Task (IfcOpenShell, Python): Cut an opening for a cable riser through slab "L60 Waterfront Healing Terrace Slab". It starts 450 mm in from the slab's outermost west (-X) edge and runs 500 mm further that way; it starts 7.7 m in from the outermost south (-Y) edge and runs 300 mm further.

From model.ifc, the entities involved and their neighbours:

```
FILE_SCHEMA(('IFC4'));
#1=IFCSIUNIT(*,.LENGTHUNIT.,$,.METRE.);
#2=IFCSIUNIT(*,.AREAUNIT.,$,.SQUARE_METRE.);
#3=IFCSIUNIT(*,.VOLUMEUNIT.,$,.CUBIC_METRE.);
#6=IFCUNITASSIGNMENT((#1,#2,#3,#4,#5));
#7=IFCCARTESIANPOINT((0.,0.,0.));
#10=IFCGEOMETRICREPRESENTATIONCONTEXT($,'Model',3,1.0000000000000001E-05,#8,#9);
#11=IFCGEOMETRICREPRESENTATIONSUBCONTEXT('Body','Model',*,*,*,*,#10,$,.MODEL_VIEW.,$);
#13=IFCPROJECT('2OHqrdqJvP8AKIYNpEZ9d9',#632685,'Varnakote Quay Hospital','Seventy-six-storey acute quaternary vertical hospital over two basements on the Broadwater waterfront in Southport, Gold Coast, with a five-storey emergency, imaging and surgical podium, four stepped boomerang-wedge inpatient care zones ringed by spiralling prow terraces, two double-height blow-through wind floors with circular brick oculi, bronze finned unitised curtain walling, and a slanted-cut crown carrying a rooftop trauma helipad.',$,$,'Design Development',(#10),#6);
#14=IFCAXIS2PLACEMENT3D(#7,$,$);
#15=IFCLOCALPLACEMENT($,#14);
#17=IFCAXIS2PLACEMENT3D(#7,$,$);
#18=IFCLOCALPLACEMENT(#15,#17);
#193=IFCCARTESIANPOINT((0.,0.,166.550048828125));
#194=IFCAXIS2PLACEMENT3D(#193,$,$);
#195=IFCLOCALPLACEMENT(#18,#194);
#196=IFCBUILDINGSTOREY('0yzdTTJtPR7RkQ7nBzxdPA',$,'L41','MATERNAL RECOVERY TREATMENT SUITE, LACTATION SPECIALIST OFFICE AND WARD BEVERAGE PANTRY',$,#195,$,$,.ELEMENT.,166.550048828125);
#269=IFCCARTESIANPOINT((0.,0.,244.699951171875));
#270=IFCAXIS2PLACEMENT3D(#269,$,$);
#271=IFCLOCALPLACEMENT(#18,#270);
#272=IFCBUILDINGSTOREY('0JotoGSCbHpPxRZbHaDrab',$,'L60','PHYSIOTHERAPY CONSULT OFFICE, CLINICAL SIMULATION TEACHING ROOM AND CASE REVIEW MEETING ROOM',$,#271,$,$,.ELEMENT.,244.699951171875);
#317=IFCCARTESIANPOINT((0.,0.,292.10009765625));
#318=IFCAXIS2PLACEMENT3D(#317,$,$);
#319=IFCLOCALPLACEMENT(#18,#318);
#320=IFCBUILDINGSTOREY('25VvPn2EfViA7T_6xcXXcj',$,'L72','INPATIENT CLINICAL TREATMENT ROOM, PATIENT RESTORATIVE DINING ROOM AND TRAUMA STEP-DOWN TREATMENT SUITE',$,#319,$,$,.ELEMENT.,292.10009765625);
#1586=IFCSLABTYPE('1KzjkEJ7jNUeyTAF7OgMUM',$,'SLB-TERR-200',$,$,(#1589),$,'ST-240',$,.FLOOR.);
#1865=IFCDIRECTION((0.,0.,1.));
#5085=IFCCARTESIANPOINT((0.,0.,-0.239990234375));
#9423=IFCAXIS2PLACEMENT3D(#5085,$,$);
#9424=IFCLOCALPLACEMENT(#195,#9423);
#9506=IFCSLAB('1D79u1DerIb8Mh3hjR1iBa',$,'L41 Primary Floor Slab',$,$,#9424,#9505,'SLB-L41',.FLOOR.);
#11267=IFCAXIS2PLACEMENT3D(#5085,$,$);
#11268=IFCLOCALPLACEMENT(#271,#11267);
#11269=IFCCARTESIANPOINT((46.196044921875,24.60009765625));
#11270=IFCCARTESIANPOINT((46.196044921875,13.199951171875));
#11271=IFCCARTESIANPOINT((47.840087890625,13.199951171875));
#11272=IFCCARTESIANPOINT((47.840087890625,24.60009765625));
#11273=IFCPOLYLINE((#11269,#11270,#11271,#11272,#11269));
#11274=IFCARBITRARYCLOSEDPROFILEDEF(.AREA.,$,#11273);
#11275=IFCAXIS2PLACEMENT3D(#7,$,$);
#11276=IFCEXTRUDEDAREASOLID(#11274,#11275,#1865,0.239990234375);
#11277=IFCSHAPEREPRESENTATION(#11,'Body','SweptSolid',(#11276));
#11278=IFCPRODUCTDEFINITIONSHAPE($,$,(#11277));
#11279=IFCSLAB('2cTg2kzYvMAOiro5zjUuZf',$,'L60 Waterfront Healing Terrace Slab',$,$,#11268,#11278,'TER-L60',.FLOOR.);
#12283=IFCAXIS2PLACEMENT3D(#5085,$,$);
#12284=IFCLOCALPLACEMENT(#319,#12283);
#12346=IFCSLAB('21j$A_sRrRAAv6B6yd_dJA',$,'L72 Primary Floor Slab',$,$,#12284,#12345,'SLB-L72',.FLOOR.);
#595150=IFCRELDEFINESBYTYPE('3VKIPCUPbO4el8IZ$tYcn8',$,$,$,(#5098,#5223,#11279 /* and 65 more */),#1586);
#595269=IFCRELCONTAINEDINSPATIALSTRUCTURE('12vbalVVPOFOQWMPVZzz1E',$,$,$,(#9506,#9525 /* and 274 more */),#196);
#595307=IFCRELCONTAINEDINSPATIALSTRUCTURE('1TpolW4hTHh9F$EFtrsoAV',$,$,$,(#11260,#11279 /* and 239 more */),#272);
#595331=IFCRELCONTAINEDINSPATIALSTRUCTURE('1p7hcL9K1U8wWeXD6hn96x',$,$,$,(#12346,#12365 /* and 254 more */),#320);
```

```python
import numpy as np
import ifcopenshell
import ifcopenshell.api.feature
import ifcopenshell.api.geometry
import ifcopenshell.api.root
import ifcopenshell.geom
import ifcopenshell.util.placement
import ifcopenshell.util.representation
import ifcopenshell.util.shape
import ifcopenshell.util.unit

model = ifcopenshell.open("model.ifc")
unit_scale = ifcopenshell.util.unit.calculate_unit_scale(model)
settings = ifcopenshell.geom.settings()


def volume(element):
    """Net volume in cubic metres, openings subtracted."""
    shape = ifcopenshell.geom.create_shape(settings, element)
    return ifcopenshell.util.shape.get_volume(shape.geometry)


slab = model.by_guid("2cTg2kzYvMAOiro5zjUuZf")
before = volume(slab)

# Extent in the slab's own axes, in metres. The edges named are its -X and -Y sides.
slab_shape = ifcopenshell.geom.create_shape(settings, slab)
vertices = ifcopenshell.util.shape.get_vertices(slab_shape.geometry)
x_min, y_min, bottom = vertices.min(axis=0)
top = vertices[:, 2].max()

opening = ifcopenshell.api.root.create_entity(model, ifc_class="IfcOpeningElement", name="Cable riser opening", predefined_type="OPENING")
context = ifcopenshell.util.representation.get_context(model, "Model", "Body", "MODEL_VIEW")
width, depth = 0.5, 0.3
outline = [(0.0, 0.0), (width, 0.0), (width, depth), (0.0, depth), (0.0, 0.0)]
# Overshoot both faces by 50 mm so the cut is clean.
shape = ifcopenshell.api.geometry.add_slab_representation(
    model, context=context, depth=top - bottom + 0.1, polyline=outline
)
ifcopenshell.api.geometry.assign_representation(model, product=opening, representation=shape)

matrix = ifcopenshell.util.placement.get_local_placement(slab.ObjectPlacement)
matrix[:, 3] = matrix @ np.append(np.array([x_min + 0.45, y_min + 7.7, bottom - 0.05]) / unit_scale, 1.0)
ifcopenshell.api.geometry.edit_object_placement(model, product=opening, matrix=matrix, is_si=False)
ifcopenshell.api.feature.add_feature(model, feature=opening, element=slab)

after = volume(slab)

print(f"slab volume {before:.3f} -> {after:.3f} m3")

model.write("model-out.ifc")
```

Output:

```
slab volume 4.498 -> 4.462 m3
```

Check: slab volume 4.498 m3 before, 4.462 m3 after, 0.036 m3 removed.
